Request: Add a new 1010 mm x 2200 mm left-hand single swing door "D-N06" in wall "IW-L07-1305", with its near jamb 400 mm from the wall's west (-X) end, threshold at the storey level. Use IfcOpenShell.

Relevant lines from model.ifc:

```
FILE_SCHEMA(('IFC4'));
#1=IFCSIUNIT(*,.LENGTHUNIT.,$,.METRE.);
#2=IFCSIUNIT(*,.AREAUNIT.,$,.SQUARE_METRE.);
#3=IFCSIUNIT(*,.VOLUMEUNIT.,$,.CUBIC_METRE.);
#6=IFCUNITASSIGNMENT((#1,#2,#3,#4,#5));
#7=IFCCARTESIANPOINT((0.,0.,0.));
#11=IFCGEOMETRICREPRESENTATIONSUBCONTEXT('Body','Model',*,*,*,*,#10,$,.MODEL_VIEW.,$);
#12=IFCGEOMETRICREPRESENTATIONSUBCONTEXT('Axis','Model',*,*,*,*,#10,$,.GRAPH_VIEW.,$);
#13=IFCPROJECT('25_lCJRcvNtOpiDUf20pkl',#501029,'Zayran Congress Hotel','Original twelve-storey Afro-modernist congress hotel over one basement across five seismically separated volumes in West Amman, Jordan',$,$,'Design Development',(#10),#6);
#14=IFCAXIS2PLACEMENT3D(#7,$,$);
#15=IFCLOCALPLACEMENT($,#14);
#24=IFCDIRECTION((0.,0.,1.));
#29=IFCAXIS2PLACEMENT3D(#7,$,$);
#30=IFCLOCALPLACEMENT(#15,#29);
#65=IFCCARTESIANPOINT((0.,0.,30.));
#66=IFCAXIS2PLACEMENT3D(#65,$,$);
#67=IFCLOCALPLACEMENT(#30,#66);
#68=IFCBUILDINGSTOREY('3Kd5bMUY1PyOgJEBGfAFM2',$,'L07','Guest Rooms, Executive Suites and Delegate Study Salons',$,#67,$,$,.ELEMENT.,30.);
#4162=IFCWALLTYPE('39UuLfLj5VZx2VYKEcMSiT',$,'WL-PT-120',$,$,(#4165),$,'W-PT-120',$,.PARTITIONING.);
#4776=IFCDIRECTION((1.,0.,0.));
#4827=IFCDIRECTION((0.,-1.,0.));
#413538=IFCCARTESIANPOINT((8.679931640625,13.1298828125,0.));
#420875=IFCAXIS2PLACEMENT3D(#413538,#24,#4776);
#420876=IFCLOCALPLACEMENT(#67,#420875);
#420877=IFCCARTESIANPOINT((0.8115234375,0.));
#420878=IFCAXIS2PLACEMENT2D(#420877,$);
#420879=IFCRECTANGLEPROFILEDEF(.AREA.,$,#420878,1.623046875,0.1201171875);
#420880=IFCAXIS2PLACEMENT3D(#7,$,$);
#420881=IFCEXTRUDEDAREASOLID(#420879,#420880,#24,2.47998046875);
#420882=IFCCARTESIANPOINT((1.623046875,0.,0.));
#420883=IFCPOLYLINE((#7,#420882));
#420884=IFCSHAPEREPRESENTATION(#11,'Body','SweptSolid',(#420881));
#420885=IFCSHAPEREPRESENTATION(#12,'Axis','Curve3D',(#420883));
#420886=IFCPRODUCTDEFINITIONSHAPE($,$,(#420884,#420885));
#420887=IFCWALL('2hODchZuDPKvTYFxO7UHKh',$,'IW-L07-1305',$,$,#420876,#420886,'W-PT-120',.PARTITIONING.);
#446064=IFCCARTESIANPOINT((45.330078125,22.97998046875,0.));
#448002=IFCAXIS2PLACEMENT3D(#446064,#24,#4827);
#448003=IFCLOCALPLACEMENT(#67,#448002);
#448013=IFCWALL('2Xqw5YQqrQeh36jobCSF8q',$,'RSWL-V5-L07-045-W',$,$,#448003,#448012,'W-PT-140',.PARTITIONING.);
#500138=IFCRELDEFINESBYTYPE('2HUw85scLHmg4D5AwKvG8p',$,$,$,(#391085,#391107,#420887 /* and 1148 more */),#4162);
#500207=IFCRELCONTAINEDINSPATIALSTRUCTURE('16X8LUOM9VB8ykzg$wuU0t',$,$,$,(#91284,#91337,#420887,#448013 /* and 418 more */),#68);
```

```python
import numpy as np
import ifcopenshell
import ifcopenshell.api.feature
import ifcopenshell.api.geometry
import ifcopenshell.api.root
import ifcopenshell.api.spatial
import ifcopenshell.geom
import ifcopenshell.util.element
import ifcopenshell.util.placement
import ifcopenshell.util.representation
import ifcopenshell.util.shape
import ifcopenshell.util.unit

model = ifcopenshell.open("model.ifc")
unit_scale = ifcopenshell.util.unit.calculate_unit_scale(model)
settings = ifcopenshell.geom.settings()


def volume(element):
    """Net volume in cubic metres, openings subtracted."""
    shape = ifcopenshell.geom.create_shape(settings, element)
    return ifcopenshell.util.shape.get_volume(shape.geometry)


wall = model.by_guid("2hODchZuDPKvTYFxO7UHKh")
storey = ifcopenshell.util.element.get_container(wall, ifc_class="IfcBuildingStorey")
context = ifcopenshell.util.representation.get_context(model, "Model", "Body", "MODEL_VIEW")
before = volume(wall)

width, height, from_end, sill = 1.01, 2.2, 0.4, 0.0  # metres

# The wall runs along its own X axis, and the end named is its -X end.
wall_shape = ifcopenshell.geom.create_shape(settings, wall)
x, y, z = ifcopenshell.util.shape.get_vertices(wall_shape.geometry).T
start = x.min() + from_end
face, thickness = float(y.min()), float(y.max() - y.min())
wall_matrix = ifcopenshell.util.placement.get_local_placement(wall.ObjectPlacement)
level = ifcopenshell.util.placement.get_local_placement(storey.ObjectPlacement)[2, 3]


def in_wall(x, y):
    """Placement at x, y metres in the wall's axes, at sill height."""
    matrix = wall_matrix.copy()
    matrix[:, 3] = wall_matrix @ np.array([x / unit_scale, y / unit_scale, 0.0, 1.0])
    matrix[2, 3] = level + sill / unit_scale
    return matrix


# Opening: a box that overshoots both wall faces by 50 mm.
opening = ifcopenshell.api.root.create_entity(model, ifc_class="IfcOpeningElement", predefined_type="OPENING")
box = ifcopenshell.api.geometry.add_wall_representation(
    model, context=context, length=width, height=height, thickness=thickness + 0.1
)
ifcopenshell.api.geometry.assign_representation(model, product=opening, representation=box)
ifcopenshell.api.geometry.edit_object_placement(model, product=opening, matrix=in_wall(start, face - 0.05), is_si=False)
ifcopenshell.api.feature.add_feature(model, feature=opening, element=wall)

door = ifcopenshell.api.root.create_entity(model, ifc_class="IfcDoor", name="D-N06", predefined_type="DOOR")
door.OverallWidth, door.OverallHeight = width / unit_scale, height / unit_scale
door.OperationType = "SINGLE_SWING_LEFT"
body = ifcopenshell.api.geometry.add_door_representation(
    model,
    context=context,
    overall_width=door.OverallWidth,
    overall_height=door.OverallHeight,
    operation_type="SINGLE_SWING_LEFT",
    lining_properties={"LiningDepth": thickness / unit_scale, "ThresholdDepth": thickness / unit_scale},
)
ifcopenshell.api.geometry.assign_representation(model, product=door, representation=body)
ifcopenshell.api.spatial.assign_container(model, products=[door], relating_structure=storey)
ifcopenshell.api.feature.add_filling(model, opening=opening, element=door)

# The lining spans the wall, so the door starts at the wall face.
ifcopenshell.api.geometry.edit_object_placement(model, product=door, matrix=in_wall(start, face), is_si=False)

after = volume(wall)

print(f"wall volume {before:.3f} -> {after:.3f} m3")

model.write("model_rev.ifc")
```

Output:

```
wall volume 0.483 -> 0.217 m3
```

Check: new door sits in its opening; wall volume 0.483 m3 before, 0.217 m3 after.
